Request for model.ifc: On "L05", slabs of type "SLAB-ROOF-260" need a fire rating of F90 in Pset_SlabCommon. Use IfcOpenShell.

First a look at what the model holds.

```python
import ifcopenshell
import ifcopenshell.util.element

model = ifcopenshell.open("model.ifc")
print(model.schema)
storey = next(s for s in model.by_type("IfcBuildingStorey") if s.Name == "L05")
slabs = [e for e in ifcopenshell.util.element.get_decomposition(storey) if e.is_a("IfcSlab")]
seen = {}
for e in slabs:
    element_type = ifcopenshell.util.element.get_type(e)
    key = (element_type.Name if element_type != e and element_type else None, ifcopenshell.util.element.get_pset(e, "Pset_SlabCommon", "FireRating"))
    seen[key] = seen.get(key, 0) + 1
for (name, value), count in sorted(seen.items(), key=str):
    print(count, "x", name, "|", value)
```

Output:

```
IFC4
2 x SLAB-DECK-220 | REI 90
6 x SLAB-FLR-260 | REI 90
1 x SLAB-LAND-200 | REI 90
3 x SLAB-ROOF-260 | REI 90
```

```python
import ifcopenshell
import ifcopenshell.api.pset
import ifcopenshell.util.element

model = ifcopenshell.open("model.ifc")

storey = next(s for s in model.by_type("IfcBuildingStorey") if s.Name == "L05")
slabs = [e for e in ifcopenshell.util.element.get_decomposition(storey) if e.is_a("IfcSlab")]

count = 0
for e in slabs:
    element_type = ifcopenshell.util.element.get_type(e)
    if element_type in (None, e) or element_type.Name != "SLAB-ROOF-260":
        continue
    # add_pset returns the element's existing set when there is one.
    pset = ifcopenshell.api.pset.add_pset(model, product=e, name="Pset_SlabCommon")
    ifcopenshell.api.pset.edit_pset(model, pset=pset, properties={"FireRating": "F90"})
    count += 1

print(count, "slabs updated")

model.write("model_edited.ifc")
```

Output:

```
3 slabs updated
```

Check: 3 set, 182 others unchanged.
